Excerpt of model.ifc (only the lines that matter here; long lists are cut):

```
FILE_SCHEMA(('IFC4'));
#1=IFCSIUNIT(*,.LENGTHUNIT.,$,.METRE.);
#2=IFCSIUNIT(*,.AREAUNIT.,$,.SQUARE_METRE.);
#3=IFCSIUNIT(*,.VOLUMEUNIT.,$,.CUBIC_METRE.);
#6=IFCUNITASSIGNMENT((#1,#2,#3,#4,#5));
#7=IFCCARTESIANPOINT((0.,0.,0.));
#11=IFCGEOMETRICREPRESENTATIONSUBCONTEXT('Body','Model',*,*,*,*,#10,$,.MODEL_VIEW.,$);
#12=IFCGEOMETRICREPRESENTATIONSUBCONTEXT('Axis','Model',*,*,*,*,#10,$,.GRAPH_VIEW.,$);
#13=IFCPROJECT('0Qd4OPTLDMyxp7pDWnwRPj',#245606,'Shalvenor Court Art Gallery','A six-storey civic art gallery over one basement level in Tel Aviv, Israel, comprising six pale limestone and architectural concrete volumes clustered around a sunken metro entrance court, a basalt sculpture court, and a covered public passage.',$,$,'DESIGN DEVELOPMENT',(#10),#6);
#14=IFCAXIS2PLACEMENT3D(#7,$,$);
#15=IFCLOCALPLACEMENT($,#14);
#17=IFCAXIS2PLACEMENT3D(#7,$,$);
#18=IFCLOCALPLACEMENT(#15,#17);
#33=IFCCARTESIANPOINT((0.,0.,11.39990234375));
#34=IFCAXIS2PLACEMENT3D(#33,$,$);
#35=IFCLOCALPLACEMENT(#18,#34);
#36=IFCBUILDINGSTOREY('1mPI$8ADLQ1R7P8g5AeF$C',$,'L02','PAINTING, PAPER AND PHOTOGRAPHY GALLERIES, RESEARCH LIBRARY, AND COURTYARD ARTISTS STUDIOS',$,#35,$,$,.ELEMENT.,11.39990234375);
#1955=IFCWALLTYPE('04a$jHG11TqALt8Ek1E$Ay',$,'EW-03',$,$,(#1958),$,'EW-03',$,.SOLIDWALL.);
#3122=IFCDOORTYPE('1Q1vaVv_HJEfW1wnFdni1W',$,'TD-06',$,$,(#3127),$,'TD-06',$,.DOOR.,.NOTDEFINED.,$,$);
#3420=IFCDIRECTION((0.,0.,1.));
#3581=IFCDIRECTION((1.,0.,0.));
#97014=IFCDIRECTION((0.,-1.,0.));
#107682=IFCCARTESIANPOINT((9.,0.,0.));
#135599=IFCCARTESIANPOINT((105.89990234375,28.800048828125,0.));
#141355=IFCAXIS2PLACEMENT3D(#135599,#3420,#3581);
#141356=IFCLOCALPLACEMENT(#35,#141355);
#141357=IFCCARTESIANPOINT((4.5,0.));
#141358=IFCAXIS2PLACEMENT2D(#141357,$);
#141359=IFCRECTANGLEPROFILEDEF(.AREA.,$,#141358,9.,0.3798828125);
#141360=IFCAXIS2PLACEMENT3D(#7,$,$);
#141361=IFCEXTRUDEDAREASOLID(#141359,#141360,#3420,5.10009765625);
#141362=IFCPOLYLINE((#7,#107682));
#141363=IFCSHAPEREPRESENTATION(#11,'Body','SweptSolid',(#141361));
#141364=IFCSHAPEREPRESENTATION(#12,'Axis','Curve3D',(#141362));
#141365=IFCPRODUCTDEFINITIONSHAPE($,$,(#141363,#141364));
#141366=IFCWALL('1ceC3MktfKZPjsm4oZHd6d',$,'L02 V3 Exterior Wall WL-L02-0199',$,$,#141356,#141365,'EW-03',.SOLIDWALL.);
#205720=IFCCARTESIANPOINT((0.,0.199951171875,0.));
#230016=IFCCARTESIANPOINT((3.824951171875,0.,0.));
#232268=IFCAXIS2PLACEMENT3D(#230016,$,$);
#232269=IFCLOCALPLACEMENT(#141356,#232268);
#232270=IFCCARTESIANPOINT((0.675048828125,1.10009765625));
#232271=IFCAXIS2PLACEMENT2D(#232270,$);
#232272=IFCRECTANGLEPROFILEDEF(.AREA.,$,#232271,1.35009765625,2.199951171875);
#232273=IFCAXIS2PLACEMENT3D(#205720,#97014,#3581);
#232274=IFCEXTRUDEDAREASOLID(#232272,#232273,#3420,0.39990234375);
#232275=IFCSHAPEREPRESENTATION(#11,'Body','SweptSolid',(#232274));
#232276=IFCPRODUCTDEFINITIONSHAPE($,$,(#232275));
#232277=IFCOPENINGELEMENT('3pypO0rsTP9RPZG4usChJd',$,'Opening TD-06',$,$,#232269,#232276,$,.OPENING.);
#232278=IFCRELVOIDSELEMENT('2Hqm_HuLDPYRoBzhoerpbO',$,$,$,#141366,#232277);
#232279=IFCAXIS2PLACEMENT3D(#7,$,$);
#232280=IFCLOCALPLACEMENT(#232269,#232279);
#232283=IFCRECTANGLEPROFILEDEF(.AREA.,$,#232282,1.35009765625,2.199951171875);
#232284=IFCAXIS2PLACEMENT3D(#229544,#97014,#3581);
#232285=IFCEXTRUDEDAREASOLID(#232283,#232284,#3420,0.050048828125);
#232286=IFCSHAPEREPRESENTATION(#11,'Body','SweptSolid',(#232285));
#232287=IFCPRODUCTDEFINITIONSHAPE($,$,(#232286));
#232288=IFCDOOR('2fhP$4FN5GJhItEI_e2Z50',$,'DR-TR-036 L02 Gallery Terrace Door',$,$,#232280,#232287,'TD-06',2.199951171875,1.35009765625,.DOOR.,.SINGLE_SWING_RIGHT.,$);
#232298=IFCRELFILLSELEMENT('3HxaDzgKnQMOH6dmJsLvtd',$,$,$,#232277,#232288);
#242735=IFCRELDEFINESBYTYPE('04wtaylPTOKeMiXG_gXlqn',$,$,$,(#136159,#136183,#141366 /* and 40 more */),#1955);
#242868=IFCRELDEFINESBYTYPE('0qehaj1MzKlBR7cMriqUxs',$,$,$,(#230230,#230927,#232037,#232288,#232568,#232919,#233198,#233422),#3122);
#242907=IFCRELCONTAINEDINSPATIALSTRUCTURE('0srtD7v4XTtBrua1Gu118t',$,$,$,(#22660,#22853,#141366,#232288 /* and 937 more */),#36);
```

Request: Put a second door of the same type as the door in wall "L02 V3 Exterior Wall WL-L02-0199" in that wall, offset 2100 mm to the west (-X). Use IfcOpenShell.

```python
import ifcopenshell
import ifcopenshell.api.feature
import ifcopenshell.api.geometry
import ifcopenshell.api.root
import ifcopenshell.geom
import ifcopenshell.util.element
import ifcopenshell.util.placement
import ifcopenshell.util.shape
import ifcopenshell.util.unit

model = ifcopenshell.open("model.ifc")
unit_scale = ifcopenshell.util.unit.calculate_unit_scale(model)
settings = ifcopenshell.geom.settings()


def volume(element):
    """Net volume in cubic metres, openings subtracted."""
    shape = ifcopenshell.geom.create_shape(settings, element)
    return ifcopenshell.util.shape.get_volume(shape.geometry)


door = model.by_id(232288)
opening = door.FillsVoids[0].RelatingOpeningElement
wall = opening.VoidsElements[0].RelatingBuildingElement
before = volume(wall)
shift = ifcopenshell.util.placement.get_local_placement(wall.ObjectPlacement)[:3, 0] * -2.1 / unit_scale

# copy_class copies the void relationship, type, container and properties, but no geometry.
new_opening = ifcopenshell.api.root.copy_class(model, product=opening)
new_opening.Representation = ifcopenshell.util.element.copy_deep(
    model, opening.Representation, exclude=["IfcGeometricRepresentationContext", "IfcRepresentationMap"]
)
new_door = ifcopenshell.api.root.copy_class(model, product=door)
new_door.Representation = ifcopenshell.util.element.copy_deep(
    model, door.Representation, exclude=["IfcGeometricRepresentationContext", "IfcRepresentationMap"]
)
new_door.Tag = None
ifcopenshell.api.feature.add_filling(model, opening=new_opening, element=new_door)

for old, new in ((opening, new_opening), (door, new_door)):
    matrix = ifcopenshell.util.placement.get_local_placement(old.ObjectPlacement)
    matrix[:3, 3] += shift
    ifcopenshell.api.geometry.edit_object_placement(model, product=new, matrix=matrix, is_si=False)

after = volume(wall)

print(f"wall volume {before:.3f} -> {after:.3f} m3")

model.write("model_edited.ifc")
```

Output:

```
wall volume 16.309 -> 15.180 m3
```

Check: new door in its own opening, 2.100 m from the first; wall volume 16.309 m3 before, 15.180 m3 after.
